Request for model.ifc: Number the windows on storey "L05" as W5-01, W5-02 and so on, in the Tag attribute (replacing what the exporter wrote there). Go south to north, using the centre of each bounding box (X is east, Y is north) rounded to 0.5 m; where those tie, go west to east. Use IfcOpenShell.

First a look at what the model holds.

```python
import ifcopenshell
import ifcopenshell.util.element
import ifcopenshell.util.placement

model = ifcopenshell.open("model.ifc")
print(model.schema)
storey = next(s for s in model.by_type("IfcBuildingStorey") if s.Name == "L05")
windows = [e for e in ifcopenshell.util.element.get_decomposition(storey) if e.is_a("IfcWindow")]
for e in sorted(windows, key=lambda e: e.id()):
    origin = ifcopenshell.util.placement.get_local_placement(e.ObjectPlacement)[:3, 3]
    print(e.id(), e.Tag, e.Name, origin.round(2) + 0.0, sep=" | ")
```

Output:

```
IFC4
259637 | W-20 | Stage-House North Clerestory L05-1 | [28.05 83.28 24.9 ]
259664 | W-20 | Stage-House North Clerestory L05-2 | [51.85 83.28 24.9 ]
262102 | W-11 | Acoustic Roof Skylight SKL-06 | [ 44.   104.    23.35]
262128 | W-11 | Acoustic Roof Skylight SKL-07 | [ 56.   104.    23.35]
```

```python
import ifcopenshell
import ifcopenshell.geom
import ifcopenshell.util.element
import ifcopenshell.util.shape

model = ifcopenshell.open("model.ifc")
settings = ifcopenshell.geom.settings()
settings.set("use-world-coords", True)


def centre(element):
    shape = ifcopenshell.geom.create_shape(settings, element)
    return ifcopenshell.util.shape.get_bbox_centroid(shape.geometry)


storey = next(s for s in model.by_type("IfcBuildingStorey") if s.Name == "L05")
windows = [e for e in ifcopenshell.util.element.get_decomposition(storey) if e.is_a("IfcWindow")]

# Insertion points can sit at a corner or the storey origin, so sort by the geometry (in metres).
centres = {e: centre(e) for e in windows}
windows.sort(key=lambda e: (round(centres[e][1] / 0.5), centres[e][0]))

for i, e in enumerate(windows, start=1):
    number = f"W5-{i:02d}"
    e.Tag = number
    print(e.id(), number)

model.write("model_rev.ifc")
```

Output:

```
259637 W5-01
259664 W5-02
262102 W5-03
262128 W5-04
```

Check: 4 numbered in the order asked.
